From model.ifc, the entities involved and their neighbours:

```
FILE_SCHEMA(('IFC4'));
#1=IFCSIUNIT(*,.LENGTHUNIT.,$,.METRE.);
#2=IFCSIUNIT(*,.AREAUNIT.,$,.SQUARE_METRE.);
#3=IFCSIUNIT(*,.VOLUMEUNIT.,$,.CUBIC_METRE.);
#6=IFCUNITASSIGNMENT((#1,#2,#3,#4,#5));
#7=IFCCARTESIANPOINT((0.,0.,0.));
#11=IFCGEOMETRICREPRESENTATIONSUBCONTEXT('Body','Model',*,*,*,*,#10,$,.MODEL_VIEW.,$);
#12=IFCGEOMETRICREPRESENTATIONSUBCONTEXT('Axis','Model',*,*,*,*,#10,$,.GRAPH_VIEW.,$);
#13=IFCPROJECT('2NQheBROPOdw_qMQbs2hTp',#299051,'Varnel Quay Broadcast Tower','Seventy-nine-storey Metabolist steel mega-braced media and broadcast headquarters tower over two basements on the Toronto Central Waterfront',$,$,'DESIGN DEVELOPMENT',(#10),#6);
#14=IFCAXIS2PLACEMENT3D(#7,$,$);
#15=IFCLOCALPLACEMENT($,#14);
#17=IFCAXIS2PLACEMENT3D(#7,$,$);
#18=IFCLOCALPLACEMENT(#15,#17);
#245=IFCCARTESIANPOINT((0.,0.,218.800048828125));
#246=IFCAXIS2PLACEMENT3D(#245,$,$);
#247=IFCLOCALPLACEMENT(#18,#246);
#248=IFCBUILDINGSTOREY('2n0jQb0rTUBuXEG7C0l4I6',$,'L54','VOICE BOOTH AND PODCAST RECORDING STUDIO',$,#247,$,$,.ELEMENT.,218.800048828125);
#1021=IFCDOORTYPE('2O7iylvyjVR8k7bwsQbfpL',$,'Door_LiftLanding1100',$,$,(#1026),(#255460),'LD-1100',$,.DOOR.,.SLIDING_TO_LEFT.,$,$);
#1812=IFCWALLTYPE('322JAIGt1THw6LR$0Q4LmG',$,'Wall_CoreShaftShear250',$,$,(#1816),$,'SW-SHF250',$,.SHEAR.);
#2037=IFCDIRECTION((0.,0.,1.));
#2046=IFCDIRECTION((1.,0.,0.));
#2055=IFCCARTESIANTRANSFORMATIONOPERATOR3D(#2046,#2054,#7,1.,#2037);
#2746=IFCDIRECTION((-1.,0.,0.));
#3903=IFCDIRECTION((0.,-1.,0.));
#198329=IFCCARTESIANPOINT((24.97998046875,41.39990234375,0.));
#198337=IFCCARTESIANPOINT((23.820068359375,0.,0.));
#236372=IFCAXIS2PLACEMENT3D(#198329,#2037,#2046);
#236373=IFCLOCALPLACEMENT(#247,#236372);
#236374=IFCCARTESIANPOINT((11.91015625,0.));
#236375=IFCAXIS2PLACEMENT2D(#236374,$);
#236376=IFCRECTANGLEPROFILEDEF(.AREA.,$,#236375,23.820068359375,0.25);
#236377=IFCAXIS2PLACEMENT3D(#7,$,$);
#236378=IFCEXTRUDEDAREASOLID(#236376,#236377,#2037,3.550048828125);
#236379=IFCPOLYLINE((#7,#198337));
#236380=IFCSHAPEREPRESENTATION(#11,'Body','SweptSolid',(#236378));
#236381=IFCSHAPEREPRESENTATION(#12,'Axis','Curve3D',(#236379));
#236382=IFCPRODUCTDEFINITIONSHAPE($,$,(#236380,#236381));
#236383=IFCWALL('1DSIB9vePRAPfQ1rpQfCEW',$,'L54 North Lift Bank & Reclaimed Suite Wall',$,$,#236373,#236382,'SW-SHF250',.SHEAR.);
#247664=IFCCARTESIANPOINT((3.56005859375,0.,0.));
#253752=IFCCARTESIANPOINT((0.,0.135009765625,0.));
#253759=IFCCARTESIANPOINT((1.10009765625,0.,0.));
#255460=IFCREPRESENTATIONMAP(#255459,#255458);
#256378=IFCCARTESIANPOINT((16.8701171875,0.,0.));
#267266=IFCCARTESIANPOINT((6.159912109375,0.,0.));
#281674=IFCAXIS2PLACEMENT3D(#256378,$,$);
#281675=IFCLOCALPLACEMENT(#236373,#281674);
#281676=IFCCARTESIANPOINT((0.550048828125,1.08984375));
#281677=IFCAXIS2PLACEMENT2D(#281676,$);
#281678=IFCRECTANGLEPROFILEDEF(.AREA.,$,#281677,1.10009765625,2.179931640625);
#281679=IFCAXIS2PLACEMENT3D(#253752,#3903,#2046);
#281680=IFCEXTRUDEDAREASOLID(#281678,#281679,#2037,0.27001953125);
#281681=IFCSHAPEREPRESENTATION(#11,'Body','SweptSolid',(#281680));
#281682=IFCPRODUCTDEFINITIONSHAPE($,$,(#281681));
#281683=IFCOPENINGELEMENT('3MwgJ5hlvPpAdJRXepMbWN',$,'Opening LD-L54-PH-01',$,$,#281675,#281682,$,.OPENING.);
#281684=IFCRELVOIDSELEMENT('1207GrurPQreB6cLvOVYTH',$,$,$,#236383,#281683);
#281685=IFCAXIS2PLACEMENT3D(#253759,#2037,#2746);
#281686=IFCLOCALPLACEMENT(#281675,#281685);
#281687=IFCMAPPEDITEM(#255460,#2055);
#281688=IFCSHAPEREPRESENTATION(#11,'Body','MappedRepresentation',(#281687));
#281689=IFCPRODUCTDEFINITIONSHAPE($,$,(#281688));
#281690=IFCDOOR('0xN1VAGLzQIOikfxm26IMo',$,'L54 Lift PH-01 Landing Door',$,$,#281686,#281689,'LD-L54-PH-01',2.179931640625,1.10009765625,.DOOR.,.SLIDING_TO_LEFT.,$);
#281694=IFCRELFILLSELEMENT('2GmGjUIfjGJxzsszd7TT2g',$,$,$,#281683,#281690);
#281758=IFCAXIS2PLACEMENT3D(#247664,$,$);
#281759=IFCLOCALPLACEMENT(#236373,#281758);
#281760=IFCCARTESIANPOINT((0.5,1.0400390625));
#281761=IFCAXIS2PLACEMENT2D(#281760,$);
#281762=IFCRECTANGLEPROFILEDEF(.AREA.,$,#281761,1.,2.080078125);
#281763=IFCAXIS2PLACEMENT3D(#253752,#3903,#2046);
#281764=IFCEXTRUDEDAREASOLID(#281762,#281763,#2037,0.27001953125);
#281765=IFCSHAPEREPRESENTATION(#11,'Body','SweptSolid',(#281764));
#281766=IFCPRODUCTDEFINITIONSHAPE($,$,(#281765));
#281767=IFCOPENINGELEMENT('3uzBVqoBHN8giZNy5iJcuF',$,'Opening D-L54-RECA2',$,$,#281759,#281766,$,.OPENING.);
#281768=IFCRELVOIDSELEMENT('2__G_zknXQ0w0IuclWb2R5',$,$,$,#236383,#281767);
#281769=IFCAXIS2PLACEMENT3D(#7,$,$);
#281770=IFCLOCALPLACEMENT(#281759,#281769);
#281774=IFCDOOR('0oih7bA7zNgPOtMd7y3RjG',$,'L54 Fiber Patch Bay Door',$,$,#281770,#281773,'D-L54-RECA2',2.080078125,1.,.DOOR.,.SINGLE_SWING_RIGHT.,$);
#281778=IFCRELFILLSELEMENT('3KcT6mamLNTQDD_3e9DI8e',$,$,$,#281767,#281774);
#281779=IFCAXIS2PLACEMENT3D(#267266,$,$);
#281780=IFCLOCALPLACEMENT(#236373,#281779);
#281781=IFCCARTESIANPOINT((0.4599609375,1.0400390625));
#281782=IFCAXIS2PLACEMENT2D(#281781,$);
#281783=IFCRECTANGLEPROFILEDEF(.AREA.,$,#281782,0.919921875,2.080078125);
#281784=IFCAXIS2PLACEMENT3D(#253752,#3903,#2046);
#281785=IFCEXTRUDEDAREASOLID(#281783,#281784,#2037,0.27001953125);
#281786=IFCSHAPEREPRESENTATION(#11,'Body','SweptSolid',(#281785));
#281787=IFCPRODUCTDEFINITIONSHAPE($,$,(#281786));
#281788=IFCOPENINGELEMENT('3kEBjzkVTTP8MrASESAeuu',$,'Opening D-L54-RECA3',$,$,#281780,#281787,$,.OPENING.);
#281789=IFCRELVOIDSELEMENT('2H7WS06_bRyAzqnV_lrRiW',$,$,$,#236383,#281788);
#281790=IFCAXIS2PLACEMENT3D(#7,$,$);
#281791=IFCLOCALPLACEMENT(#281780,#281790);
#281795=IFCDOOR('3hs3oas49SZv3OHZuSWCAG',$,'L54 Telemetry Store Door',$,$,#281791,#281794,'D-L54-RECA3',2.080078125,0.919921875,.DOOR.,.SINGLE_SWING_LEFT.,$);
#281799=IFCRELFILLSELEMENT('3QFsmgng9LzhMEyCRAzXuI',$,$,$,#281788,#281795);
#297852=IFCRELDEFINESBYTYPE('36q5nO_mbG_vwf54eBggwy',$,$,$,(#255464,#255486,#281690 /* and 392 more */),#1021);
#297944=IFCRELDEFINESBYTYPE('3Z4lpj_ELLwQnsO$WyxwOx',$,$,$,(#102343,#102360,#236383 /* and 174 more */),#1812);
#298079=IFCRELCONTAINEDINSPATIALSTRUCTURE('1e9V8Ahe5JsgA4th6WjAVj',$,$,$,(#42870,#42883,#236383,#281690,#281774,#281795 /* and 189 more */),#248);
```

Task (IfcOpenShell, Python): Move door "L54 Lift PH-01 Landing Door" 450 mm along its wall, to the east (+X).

```python
import ifcopenshell
import ifcopenshell.api.geometry
import ifcopenshell.util.placement

model = ifcopenshell.open("model.ifc")

door = model.by_guid("0xN1VAGLzQIOikfxm26IMo")
opening = door.FillsVoids[0].RelatingOpeningElement
wall = opening.VoidsElements[0].RelatingBuildingElement

wall_matrix = ifcopenshell.util.placement.get_local_placement(wall.ObjectPlacement)
shift = wall_matrix[:3, 0] * 0.45
before = ifcopenshell.util.placement.get_local_placement(door.ObjectPlacement)[:3, 3].copy()

# The door is placed relative to its opening, so it follows when the opening moves.
matrix = ifcopenshell.util.placement.get_local_placement(opening.ObjectPlacement)
matrix[:3, 3] += shift
ifcopenshell.api.geometry.edit_object_placement(
    model, product=opening, matrix=matrix, is_si=False, should_transform_children=True
)

after = ifcopenshell.util.placement.get_local_placement(door.ObjectPlacement)[:3, 3]
print("door moved by", (after - before).round(3) + 0.0)

model.write("model-out.ifc")
```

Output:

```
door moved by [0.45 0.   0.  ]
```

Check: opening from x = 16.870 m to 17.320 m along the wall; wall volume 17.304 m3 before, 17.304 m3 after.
